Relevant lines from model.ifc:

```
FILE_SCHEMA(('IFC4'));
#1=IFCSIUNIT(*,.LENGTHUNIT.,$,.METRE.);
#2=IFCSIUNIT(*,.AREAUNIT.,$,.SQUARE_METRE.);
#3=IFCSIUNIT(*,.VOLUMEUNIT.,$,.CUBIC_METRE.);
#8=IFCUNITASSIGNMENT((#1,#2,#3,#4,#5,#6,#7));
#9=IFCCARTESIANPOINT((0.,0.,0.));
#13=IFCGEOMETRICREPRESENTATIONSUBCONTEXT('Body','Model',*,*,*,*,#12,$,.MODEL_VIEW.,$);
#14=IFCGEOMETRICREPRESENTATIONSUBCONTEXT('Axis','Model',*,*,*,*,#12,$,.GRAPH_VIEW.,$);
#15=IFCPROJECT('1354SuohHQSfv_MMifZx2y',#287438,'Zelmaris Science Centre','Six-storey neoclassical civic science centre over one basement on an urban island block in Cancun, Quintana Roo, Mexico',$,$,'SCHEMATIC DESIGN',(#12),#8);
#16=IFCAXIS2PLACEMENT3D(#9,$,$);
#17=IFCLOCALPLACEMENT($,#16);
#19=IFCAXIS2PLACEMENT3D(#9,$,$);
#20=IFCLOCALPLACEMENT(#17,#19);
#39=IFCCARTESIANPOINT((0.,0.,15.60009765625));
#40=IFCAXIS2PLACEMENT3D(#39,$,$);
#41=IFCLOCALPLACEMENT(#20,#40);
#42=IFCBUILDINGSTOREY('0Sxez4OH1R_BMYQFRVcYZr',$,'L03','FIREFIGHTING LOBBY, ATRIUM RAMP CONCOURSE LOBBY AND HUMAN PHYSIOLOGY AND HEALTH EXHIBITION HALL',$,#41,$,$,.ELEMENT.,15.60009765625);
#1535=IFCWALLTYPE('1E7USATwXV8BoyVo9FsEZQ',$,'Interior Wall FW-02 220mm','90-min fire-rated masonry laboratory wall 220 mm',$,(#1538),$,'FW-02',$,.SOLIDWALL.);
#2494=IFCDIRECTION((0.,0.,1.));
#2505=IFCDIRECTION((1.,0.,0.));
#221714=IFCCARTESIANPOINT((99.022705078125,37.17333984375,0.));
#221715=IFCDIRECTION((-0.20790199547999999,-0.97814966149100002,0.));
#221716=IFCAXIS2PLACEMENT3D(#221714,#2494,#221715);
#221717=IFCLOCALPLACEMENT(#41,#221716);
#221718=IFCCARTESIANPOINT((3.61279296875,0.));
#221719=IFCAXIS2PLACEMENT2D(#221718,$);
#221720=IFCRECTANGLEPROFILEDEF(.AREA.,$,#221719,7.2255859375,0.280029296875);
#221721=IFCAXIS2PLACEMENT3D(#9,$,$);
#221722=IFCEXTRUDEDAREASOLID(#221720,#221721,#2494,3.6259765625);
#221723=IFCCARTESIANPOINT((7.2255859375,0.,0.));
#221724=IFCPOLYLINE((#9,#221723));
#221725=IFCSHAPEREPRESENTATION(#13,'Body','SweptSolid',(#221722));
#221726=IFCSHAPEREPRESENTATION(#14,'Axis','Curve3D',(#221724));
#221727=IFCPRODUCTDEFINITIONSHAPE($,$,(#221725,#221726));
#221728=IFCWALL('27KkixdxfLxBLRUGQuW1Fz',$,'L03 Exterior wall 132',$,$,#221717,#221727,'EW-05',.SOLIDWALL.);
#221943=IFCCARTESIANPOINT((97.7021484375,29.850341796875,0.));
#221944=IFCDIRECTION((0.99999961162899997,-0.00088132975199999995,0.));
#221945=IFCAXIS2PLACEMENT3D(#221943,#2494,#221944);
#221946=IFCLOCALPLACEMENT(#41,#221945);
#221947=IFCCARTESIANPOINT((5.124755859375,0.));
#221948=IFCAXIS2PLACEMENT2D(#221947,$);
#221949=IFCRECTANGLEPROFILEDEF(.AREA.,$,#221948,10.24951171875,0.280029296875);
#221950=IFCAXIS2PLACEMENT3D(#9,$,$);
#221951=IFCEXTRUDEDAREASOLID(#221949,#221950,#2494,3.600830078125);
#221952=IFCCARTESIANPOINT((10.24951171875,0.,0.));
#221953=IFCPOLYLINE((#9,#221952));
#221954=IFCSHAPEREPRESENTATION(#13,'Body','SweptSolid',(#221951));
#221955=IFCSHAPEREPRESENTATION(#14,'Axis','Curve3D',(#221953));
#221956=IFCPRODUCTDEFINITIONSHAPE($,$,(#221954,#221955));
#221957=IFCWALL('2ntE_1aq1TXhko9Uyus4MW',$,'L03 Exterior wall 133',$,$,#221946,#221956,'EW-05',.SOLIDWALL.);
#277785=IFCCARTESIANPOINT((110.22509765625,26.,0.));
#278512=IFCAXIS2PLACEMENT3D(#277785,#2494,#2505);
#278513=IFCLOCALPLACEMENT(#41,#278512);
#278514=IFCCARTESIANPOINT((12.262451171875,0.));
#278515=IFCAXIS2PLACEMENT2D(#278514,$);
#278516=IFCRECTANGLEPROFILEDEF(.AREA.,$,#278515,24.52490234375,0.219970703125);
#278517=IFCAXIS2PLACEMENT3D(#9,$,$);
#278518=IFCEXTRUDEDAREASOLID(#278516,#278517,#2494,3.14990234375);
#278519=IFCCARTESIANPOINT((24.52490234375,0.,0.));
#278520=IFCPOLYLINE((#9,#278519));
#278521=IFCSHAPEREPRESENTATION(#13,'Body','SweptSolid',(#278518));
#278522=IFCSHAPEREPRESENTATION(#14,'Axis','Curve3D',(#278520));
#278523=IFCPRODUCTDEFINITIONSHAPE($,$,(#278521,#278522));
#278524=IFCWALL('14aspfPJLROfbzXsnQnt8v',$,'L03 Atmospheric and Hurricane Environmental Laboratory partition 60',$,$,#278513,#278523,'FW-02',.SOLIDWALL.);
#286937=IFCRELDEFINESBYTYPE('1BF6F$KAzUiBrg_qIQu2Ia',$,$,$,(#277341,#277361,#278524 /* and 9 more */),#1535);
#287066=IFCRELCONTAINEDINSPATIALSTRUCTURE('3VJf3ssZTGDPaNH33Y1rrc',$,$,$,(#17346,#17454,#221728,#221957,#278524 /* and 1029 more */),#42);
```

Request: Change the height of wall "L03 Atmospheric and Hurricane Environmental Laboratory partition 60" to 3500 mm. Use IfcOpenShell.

```python
import ifcopenshell
import ifcopenshell.geom
import ifcopenshell.util.representation
import ifcopenshell.util.shape

model = ifcopenshell.open("model.ifc")
settings = ifcopenshell.geom.settings()


def volume(element):
    """Net volume in cubic metres, openings subtracted."""
    shape = ifcopenshell.geom.create_shape(settings, element)
    return ifcopenshell.util.shape.get_volume(shape.geometry)


wall = model.by_guid("14aspfPJLROfbzXsnQnt8v")
before = volume(wall)

body = ifcopenshell.util.representation.get_representation(wall, "Model", "Body")
solid = body.Items[0]
old_height = solid.Depth
solid.Depth = 3.5
after = volume(wall)

print(f"height {old_height:g} -> {solid.Depth:g}, volume {before:.3f} -> {after:.3f} m3")

model.write("model-out.ifc")
```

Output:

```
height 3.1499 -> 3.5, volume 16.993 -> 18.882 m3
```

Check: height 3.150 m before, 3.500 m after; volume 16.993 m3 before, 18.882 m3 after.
